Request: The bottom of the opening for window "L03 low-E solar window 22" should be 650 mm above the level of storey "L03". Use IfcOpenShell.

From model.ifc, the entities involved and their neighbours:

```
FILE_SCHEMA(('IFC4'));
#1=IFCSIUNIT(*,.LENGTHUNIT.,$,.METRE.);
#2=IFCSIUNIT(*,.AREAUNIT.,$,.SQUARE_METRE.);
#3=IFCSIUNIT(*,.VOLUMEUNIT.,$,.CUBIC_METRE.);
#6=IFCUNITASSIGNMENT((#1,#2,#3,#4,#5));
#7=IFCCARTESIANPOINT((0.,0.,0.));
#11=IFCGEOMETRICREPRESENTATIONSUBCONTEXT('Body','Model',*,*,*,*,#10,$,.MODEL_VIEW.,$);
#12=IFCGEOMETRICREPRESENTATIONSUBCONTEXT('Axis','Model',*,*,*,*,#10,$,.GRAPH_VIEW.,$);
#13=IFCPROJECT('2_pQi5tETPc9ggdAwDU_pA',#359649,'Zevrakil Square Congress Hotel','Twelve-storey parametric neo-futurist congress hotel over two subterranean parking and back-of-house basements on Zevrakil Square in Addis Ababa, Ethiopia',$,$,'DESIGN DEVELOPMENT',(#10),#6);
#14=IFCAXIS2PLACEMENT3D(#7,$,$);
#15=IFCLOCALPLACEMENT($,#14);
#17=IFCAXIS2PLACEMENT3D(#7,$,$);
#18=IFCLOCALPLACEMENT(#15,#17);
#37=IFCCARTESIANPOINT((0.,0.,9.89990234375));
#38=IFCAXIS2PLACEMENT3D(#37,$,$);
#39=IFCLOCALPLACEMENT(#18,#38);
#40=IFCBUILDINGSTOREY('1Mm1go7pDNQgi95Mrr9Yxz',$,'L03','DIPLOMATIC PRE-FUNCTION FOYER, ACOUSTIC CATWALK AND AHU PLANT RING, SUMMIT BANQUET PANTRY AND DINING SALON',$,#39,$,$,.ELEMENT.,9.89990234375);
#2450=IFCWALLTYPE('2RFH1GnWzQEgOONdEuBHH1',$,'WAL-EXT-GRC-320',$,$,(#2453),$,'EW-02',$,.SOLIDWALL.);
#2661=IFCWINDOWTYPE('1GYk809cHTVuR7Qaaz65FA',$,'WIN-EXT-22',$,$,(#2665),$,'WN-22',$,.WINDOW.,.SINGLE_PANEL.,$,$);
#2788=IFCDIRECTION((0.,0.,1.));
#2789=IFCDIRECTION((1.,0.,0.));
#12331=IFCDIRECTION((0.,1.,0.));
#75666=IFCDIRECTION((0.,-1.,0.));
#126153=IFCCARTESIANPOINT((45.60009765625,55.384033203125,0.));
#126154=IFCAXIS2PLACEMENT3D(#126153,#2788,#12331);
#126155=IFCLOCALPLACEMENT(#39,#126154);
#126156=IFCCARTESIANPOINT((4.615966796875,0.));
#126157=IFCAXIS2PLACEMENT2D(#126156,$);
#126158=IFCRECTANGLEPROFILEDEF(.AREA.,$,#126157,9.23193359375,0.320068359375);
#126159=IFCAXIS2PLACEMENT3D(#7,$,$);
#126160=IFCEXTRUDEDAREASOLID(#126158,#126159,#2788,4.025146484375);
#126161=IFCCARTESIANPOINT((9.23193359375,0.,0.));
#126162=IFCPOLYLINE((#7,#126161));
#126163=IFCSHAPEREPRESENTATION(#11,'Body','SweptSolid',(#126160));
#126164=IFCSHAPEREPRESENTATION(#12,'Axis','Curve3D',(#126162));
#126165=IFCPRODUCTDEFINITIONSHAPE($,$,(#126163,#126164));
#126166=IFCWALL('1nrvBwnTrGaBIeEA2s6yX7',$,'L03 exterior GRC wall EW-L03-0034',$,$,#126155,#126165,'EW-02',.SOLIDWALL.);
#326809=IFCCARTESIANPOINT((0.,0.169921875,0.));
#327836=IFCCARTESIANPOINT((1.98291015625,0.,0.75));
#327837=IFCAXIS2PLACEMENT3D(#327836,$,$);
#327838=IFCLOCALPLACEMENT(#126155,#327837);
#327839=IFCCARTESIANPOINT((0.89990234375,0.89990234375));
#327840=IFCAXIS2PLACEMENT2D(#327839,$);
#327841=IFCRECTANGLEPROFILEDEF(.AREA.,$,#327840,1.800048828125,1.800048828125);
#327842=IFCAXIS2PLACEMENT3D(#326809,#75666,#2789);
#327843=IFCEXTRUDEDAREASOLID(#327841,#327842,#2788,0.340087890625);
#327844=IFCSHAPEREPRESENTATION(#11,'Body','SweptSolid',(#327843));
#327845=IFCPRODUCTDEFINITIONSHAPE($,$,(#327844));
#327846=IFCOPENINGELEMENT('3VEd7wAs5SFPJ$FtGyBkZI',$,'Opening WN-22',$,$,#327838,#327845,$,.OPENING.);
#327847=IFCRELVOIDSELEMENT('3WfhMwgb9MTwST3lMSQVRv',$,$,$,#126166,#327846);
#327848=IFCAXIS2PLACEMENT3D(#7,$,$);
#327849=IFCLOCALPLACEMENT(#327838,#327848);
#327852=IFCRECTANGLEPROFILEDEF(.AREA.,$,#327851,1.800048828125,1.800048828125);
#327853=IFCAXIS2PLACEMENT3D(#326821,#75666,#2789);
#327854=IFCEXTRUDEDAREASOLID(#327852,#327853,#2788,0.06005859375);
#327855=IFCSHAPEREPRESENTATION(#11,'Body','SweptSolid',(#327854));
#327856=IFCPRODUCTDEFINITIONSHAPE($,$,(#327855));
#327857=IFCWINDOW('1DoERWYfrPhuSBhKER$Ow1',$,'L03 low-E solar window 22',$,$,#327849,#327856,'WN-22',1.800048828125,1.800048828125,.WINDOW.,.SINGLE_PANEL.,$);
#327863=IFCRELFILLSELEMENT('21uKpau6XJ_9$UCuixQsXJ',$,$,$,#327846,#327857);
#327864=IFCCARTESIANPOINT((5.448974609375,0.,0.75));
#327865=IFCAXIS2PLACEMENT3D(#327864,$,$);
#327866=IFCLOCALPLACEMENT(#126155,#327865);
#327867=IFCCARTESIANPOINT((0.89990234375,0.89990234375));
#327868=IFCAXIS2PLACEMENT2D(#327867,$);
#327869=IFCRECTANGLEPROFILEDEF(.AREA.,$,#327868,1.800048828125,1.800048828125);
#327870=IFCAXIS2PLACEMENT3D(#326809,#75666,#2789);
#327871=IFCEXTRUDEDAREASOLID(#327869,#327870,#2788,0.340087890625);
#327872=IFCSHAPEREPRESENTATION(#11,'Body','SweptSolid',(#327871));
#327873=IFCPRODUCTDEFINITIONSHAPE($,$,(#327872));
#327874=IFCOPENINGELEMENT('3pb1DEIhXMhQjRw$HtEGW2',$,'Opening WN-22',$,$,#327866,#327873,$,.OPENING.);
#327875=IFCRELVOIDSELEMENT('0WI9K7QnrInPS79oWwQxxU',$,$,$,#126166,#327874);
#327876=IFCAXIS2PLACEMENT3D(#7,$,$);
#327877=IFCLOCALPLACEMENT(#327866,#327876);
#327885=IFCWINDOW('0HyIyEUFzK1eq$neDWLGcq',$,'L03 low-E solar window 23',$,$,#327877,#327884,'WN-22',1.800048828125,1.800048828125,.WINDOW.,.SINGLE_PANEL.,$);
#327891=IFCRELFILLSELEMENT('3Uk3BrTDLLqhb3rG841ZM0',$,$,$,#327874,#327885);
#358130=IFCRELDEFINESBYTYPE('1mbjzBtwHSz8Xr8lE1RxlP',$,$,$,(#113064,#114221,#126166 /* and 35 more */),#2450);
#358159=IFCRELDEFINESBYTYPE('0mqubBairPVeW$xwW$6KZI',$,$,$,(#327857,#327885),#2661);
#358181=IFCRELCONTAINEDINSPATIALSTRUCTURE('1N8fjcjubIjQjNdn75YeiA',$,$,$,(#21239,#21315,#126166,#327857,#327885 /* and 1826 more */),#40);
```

```python
import numpy as np
import ifcopenshell
import ifcopenshell.api.geometry
import ifcopenshell.geom
import ifcopenshell.util.element
import ifcopenshell.util.placement
import ifcopenshell.util.shape
import ifcopenshell.util.unit

model = ifcopenshell.open("model.ifc")
unit_scale = ifcopenshell.util.unit.calculate_unit_scale(model)

window = model.by_guid("1DoERWYfrPhuSBhKER$Ow1")
opening = window.FillsVoids[0].RelatingOpeningElement
storey = ifcopenshell.util.element.get_container(window, ifc_class="IfcBuildingStorey")
level = ifcopenshell.util.placement.get_local_placement(storey.ObjectPlacement)[2, 3]

# The opening's origin need not be at the sill, so measure its lowest point.
shape = ifcopenshell.geom.create_shape(ifcopenshell.geom.settings(), opening)
bottom = ifcopenshell.util.shape.get_shape_bottom_elevation(shape, shape.geometry) / unit_scale
dz = level + 0.65 - bottom

shift = np.array([0.0, 0.0, dz])
# The window is placed relative to its opening, so it follows when the opening moves.
matrix = ifcopenshell.util.placement.get_local_placement(opening.ObjectPlacement)
matrix[:3, 3] += shift
ifcopenshell.api.geometry.edit_object_placement(
    model, product=opening, matrix=matrix, is_si=False, should_transform_children=True
)

print(f"moved by {dz * unit_scale:+.3f} m")

model.write("model_updated.ifc")
```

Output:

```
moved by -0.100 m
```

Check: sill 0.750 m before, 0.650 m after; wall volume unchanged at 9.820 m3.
